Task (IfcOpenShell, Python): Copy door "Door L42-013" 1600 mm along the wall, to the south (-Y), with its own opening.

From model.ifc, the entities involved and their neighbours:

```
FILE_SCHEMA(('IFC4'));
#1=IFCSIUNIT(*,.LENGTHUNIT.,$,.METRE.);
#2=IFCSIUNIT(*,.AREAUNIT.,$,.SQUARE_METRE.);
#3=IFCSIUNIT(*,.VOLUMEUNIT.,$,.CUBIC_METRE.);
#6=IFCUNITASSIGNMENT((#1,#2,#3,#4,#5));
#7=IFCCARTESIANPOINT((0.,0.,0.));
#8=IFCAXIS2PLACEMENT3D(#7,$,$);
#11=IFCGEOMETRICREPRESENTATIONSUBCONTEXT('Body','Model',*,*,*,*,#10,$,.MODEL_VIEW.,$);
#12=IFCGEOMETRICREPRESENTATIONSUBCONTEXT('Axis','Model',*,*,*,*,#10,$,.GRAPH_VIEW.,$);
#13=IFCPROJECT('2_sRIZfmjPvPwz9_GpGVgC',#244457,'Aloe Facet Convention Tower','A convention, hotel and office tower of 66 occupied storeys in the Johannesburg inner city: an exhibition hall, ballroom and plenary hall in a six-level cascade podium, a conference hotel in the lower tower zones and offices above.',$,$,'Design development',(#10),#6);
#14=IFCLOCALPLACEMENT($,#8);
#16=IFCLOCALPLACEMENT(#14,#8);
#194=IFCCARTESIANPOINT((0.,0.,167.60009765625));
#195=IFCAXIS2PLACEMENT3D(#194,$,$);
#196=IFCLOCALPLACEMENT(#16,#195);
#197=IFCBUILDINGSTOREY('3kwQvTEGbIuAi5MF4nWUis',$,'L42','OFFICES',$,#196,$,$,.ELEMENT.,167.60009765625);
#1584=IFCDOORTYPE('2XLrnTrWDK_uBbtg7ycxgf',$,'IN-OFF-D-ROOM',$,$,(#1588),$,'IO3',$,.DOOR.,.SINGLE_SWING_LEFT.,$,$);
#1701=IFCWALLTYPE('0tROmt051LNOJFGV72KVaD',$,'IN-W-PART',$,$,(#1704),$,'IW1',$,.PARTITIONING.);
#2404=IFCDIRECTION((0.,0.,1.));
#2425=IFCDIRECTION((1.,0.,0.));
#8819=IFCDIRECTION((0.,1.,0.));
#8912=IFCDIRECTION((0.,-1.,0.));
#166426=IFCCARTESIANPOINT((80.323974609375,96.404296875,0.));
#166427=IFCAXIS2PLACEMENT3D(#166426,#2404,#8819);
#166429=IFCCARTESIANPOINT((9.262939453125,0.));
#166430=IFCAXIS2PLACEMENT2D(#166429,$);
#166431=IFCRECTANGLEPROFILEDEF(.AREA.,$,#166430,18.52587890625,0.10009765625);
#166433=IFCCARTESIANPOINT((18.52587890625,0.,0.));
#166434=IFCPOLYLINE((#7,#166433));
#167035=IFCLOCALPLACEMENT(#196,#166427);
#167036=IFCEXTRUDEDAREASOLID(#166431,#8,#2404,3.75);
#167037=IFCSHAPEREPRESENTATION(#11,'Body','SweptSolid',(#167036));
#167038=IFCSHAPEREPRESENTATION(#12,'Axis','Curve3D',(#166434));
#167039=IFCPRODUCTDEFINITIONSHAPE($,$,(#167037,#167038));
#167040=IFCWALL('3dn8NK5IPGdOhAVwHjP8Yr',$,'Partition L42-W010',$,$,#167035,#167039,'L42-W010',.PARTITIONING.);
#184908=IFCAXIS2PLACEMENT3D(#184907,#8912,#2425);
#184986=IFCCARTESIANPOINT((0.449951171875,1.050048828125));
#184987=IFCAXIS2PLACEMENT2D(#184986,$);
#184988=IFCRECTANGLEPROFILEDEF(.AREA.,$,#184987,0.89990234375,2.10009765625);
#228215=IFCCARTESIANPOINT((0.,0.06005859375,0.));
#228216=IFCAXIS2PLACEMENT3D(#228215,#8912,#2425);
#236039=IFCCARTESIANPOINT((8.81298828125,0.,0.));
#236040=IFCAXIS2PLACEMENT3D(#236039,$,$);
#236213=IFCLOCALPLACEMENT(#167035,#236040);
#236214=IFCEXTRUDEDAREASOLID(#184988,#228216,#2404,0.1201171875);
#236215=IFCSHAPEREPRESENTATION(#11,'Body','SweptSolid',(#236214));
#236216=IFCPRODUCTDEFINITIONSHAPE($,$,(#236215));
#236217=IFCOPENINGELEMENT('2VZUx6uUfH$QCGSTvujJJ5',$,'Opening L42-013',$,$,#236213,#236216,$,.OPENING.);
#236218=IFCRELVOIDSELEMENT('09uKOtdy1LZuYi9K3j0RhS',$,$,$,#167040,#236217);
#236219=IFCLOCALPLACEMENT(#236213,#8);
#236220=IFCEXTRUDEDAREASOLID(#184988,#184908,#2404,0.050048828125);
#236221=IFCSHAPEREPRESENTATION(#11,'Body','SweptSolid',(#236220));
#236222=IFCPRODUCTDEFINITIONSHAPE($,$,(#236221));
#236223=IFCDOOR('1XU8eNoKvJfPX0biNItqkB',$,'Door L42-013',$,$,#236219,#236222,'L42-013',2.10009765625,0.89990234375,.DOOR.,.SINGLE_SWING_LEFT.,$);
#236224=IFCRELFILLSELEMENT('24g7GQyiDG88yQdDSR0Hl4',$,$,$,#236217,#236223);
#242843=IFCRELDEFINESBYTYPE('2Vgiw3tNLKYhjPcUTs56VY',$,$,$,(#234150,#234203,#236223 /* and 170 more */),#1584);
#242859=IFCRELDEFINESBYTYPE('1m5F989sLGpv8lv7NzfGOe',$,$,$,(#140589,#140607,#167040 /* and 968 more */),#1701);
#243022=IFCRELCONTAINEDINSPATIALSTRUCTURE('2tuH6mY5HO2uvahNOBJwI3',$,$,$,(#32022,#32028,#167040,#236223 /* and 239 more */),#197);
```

```python
import ifcopenshell
import ifcopenshell.api.feature
import ifcopenshell.api.geometry
import ifcopenshell.api.root
import ifcopenshell.geom
import ifcopenshell.util.element
import ifcopenshell.util.placement
import ifcopenshell.util.shape
import ifcopenshell.util.unit

model = ifcopenshell.open("model.ifc")
unit_scale = ifcopenshell.util.unit.calculate_unit_scale(model)
settings = ifcopenshell.geom.settings()


def volume(element):
    """Net volume in cubic metres, openings subtracted."""
    shape = ifcopenshell.geom.create_shape(settings, element)
    return ifcopenshell.util.shape.get_volume(shape.geometry)


door = model.by_guid("1XU8eNoKvJfPX0biNItqkB")
opening = door.FillsVoids[0].RelatingOpeningElement
wall = opening.VoidsElements[0].RelatingBuildingElement
before = volume(wall)
shift = ifcopenshell.util.placement.get_local_placement(wall.ObjectPlacement)[:3, 0] * -1.6 / unit_scale

# copy_class copies the void relationship, type, container and properties, but no geometry.
new_opening = ifcopenshell.api.root.copy_class(model, product=opening)
new_opening.Representation = ifcopenshell.util.element.copy_deep(
    model, opening.Representation, exclude=["IfcGeometricRepresentationContext", "IfcRepresentationMap"]
)
new_door = ifcopenshell.api.root.copy_class(model, product=door)
new_door.Representation = ifcopenshell.util.element.copy_deep(
    model, door.Representation, exclude=["IfcGeometricRepresentationContext", "IfcRepresentationMap"]
)
new_door.Tag = None
ifcopenshell.api.feature.add_filling(model, opening=new_opening, element=new_door)

for old, new in ((opening, new_opening), (door, new_door)):
    matrix = ifcopenshell.util.placement.get_local_placement(old.ObjectPlacement)
    matrix[:3, 3] += shift
    ifcopenshell.api.geometry.edit_object_placement(model, product=new, matrix=matrix, is_si=False)

after = volume(wall)

print(f"wall volume {before:.3f} -> {after:.3f} m3")

model.write("model-out.ifc")
```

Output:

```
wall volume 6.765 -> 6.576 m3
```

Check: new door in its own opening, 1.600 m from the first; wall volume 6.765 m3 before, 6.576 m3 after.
